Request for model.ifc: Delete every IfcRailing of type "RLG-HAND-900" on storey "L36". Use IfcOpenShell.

First a look at what the model holds.

```python
import ifcopenshell
import ifcopenshell.util.element

model = ifcopenshell.open("model.ifc")
print(model.schema)
storey = next(s for s in model.by_type("IfcBuildingStorey") if s.Name == "L36")
railings = [e for e in ifcopenshell.util.element.get_decomposition(storey) if e.is_a("IfcRailing")]
seen = {}
for e in railings:
    element_type = ifcopenshell.util.element.get_type(e)
    name = element_type.Name if element_type not in (None, e) else None
    seen[name] = seen.get(name, 0) + 1
for name, count in sorted(seen.items(), key=str):
    print(count, "x", name)
```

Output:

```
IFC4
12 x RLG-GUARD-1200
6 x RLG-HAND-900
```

```python
import ifcopenshell
import ifcopenshell.api.root
import ifcopenshell.util.element

model = ifcopenshell.open("model.ifc")

storey = next(s for s in model.by_type("IfcBuildingStorey") if s.Name == "L36")
railings = [e for e in ifcopenshell.util.element.get_decomposition(storey) if e.is_a("IfcRailing")]
targets = [e for e in railings if (t := ifcopenshell.util.element.get_type(e)) not in (None, e) and t.Name == "RLG-HAND-900"]

for e in targets:
    ifcopenshell.api.root.remove_product(model, product=e)
print(len(targets), "removed")

model.write("model_v2.ifc")
```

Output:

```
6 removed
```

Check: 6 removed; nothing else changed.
